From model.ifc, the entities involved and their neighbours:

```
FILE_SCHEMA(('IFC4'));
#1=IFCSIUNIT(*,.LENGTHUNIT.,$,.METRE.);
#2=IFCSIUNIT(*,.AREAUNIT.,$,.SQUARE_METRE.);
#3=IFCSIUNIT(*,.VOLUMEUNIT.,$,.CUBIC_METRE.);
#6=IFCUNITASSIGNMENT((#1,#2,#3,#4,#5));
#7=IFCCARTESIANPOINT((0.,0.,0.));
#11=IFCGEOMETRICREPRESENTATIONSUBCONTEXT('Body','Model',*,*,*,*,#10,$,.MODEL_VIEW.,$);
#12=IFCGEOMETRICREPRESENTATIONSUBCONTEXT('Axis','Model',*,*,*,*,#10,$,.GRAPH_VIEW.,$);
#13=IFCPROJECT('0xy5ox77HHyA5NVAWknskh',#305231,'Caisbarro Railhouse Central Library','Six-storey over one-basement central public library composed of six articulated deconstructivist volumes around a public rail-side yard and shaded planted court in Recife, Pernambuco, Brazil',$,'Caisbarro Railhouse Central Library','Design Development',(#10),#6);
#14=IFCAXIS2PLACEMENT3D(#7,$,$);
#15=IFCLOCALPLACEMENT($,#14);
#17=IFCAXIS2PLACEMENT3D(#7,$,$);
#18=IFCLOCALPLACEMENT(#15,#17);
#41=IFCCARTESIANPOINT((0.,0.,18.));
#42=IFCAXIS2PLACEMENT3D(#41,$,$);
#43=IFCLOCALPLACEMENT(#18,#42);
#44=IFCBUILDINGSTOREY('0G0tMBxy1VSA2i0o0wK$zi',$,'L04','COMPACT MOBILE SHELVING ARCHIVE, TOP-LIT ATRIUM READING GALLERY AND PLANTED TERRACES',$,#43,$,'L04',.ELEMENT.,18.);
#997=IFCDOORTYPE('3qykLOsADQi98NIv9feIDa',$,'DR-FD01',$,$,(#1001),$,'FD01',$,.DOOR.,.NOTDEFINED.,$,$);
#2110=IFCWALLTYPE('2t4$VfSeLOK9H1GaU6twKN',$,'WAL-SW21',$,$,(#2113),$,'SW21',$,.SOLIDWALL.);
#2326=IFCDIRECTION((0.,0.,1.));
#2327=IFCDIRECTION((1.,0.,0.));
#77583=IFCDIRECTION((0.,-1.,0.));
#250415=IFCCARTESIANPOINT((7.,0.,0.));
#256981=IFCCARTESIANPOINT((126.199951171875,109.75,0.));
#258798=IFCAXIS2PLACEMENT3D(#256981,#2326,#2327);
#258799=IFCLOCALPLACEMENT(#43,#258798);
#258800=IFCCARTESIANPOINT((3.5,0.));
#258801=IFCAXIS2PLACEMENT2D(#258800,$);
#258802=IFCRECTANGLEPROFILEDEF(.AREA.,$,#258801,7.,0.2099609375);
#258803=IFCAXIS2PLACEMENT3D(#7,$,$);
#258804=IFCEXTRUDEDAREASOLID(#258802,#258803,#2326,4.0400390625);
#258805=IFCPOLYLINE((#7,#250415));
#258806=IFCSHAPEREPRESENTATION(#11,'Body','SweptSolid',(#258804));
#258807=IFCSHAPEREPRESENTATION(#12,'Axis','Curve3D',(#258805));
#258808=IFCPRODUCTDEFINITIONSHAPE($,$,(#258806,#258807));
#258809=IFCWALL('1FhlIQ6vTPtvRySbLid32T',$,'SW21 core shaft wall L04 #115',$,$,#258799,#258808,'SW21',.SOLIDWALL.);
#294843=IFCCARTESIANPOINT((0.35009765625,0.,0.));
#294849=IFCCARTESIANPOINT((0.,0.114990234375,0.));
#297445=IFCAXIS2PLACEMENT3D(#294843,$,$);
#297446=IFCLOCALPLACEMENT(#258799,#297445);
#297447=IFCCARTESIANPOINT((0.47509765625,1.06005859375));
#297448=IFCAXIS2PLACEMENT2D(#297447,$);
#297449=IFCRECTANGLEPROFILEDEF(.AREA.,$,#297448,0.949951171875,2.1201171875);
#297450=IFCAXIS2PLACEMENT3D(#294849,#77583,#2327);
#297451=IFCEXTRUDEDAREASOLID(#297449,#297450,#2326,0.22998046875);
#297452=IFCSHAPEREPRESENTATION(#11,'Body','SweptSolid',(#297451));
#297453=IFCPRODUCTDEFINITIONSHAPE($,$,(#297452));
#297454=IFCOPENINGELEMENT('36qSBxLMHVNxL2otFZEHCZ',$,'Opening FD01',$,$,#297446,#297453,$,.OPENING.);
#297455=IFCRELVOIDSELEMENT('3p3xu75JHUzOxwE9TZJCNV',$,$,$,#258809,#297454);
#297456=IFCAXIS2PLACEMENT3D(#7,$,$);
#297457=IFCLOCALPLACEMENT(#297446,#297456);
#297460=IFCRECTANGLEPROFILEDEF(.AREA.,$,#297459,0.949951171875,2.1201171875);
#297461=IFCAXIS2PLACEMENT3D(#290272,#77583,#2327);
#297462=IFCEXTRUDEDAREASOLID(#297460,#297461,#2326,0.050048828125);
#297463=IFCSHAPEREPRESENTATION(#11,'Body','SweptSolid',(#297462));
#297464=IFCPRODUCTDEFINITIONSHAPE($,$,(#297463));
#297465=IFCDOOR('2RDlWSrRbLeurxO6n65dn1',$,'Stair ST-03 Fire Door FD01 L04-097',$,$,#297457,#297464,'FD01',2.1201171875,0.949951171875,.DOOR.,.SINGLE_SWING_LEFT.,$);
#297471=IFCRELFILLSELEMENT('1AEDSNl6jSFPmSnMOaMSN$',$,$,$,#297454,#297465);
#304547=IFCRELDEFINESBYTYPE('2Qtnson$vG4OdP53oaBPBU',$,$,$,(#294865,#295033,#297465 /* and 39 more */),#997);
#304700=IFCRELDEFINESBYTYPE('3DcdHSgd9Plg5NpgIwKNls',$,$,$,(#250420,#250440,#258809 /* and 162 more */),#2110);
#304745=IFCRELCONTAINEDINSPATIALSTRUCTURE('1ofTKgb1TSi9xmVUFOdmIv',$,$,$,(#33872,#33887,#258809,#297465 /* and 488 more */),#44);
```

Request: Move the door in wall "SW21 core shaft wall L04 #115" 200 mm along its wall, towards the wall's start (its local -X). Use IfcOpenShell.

```python
import ifcopenshell
import ifcopenshell.api.geometry
import ifcopenshell.util.placement
import ifcopenshell.util.unit

model = ifcopenshell.open("model.ifc")
unit_scale = ifcopenshell.util.unit.calculate_unit_scale(model)

door = model.by_guid("2RDlWSrRbLeurxO6n65dn1")
opening = door.FillsVoids[0].RelatingOpeningElement
wall = opening.VoidsElements[0].RelatingBuildingElement

wall_matrix = ifcopenshell.util.placement.get_local_placement(wall.ObjectPlacement)
shift = wall_matrix[:3, 0] * -0.2 / unit_scale
before = ifcopenshell.util.placement.get_local_placement(door.ObjectPlacement)[:3, 3].copy()

# The door is placed relative to its opening, so it follows when the opening moves.
matrix = ifcopenshell.util.placement.get_local_placement(opening.ObjectPlacement)
matrix[:3, 3] += shift
ifcopenshell.api.geometry.edit_object_placement(
    model, product=opening, matrix=matrix, is_si=False, should_transform_children=True
)

after = ifcopenshell.util.placement.get_local_placement(door.ObjectPlacement)[:3, 3]
print("door moved by", (after - before).round(3) + 0.0)

model.write("model_edited.ifc")
```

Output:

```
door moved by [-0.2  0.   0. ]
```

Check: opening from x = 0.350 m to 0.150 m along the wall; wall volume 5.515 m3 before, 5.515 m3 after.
